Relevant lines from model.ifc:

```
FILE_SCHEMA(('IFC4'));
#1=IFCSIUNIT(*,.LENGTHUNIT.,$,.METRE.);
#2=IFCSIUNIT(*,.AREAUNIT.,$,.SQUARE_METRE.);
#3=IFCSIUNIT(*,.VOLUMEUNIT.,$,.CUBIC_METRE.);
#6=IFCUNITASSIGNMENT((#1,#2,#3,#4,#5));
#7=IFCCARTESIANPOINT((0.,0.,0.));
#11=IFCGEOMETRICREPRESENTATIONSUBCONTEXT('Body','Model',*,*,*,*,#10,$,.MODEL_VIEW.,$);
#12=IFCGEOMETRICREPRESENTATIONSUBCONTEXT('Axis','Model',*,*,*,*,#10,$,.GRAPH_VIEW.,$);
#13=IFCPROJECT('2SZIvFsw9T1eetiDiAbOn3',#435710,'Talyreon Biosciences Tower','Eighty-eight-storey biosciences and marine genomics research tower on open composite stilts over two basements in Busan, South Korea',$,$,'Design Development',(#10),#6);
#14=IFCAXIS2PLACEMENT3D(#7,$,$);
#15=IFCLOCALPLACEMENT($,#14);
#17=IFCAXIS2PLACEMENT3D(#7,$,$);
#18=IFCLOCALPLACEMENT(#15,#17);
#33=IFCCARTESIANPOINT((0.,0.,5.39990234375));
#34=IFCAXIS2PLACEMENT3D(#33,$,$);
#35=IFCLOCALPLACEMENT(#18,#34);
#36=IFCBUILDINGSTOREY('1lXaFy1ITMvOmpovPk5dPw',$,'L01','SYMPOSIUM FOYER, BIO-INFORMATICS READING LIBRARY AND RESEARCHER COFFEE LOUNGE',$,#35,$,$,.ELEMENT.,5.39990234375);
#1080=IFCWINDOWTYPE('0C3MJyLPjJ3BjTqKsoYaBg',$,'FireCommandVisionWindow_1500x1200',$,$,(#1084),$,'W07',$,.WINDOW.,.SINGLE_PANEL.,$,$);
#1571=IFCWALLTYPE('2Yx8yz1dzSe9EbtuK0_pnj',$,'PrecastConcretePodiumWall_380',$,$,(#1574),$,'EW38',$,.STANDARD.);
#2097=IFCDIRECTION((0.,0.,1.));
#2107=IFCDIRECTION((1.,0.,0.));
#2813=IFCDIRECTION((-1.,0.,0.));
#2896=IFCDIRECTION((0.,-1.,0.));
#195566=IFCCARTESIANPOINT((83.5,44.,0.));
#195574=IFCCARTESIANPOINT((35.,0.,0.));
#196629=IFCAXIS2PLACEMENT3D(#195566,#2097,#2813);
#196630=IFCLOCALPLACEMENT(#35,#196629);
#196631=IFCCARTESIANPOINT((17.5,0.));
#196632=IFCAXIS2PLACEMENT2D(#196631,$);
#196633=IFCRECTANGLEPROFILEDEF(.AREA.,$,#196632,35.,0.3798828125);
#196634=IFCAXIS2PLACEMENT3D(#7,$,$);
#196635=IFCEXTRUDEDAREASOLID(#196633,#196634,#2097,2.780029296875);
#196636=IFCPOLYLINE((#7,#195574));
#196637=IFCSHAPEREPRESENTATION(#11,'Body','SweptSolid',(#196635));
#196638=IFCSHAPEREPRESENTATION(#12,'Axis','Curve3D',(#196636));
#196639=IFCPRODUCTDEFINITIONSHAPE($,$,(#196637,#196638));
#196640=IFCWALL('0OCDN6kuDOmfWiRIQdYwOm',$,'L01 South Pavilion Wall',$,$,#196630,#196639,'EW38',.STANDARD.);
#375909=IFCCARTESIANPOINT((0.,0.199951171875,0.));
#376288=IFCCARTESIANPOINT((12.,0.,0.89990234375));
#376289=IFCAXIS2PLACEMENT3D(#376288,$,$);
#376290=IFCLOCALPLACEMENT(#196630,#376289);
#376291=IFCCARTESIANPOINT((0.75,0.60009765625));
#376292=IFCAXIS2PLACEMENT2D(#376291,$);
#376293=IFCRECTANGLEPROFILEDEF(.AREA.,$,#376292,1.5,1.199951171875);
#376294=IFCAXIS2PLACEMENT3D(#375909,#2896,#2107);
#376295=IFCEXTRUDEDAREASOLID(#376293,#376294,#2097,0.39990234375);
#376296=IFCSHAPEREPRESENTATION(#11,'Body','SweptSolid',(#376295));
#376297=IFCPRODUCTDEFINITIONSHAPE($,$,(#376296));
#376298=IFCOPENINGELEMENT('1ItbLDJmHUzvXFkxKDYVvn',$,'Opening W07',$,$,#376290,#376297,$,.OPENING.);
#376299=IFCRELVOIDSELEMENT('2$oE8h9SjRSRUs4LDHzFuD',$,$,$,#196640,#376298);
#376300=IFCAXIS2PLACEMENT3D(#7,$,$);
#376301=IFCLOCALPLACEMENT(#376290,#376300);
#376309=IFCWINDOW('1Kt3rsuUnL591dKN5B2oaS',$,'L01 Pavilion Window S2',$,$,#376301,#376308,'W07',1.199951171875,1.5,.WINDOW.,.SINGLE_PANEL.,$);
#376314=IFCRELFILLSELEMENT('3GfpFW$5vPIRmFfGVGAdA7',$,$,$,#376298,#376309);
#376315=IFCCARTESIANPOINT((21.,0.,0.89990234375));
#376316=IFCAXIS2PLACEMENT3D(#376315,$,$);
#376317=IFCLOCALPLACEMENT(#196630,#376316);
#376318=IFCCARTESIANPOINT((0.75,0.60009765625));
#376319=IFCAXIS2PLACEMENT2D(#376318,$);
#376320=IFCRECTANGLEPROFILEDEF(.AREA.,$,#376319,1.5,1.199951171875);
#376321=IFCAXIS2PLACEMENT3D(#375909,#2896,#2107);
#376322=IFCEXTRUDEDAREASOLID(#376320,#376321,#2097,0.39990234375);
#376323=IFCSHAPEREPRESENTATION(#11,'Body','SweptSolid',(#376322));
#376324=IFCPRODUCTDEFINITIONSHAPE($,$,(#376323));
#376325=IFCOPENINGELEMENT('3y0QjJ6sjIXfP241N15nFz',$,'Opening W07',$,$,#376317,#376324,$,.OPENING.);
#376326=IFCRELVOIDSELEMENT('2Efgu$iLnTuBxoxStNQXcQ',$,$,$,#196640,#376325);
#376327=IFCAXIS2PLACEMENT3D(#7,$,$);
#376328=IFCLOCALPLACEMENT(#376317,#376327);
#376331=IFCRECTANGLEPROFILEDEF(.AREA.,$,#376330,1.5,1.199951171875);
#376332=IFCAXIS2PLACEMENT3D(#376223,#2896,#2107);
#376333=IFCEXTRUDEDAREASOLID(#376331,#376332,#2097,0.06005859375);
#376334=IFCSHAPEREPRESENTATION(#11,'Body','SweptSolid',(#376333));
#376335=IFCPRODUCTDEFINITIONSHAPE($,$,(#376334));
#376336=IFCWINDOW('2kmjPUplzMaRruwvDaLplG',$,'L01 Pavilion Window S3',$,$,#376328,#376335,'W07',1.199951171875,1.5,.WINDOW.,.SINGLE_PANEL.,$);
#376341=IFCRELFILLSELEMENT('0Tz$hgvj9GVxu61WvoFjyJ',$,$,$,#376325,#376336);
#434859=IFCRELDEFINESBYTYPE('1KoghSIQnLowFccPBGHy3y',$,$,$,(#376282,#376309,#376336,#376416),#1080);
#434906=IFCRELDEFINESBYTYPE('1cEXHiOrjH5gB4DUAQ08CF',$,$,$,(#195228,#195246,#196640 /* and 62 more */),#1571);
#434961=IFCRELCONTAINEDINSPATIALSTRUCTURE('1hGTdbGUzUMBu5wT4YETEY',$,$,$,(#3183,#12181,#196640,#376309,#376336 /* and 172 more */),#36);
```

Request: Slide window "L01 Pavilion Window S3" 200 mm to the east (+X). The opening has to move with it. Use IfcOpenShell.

```python
import ifcopenshell
import ifcopenshell.api.geometry
import ifcopenshell.util.placement

model = ifcopenshell.open("model.ifc")

window = model.by_guid("2kmjPUplzMaRruwvDaLplG")
opening = window.FillsVoids[0].RelatingOpeningElement
wall = opening.VoidsElements[0].RelatingBuildingElement

wall_matrix = ifcopenshell.util.placement.get_local_placement(wall.ObjectPlacement)
shift = wall_matrix[:3, 0] * -0.2
before = ifcopenshell.util.placement.get_local_placement(window.ObjectPlacement)[:3, 3].copy()

# The window is placed relative to its opening, so it follows when the opening moves.
matrix = ifcopenshell.util.placement.get_local_placement(opening.ObjectPlacement)
matrix[:3, 3] += shift
ifcopenshell.api.geometry.edit_object_placement(
    model, product=opening, matrix=matrix, is_si=False, should_transform_children=True
)

after = ifcopenshell.util.placement.get_local_placement(window.ObjectPlacement)[:3, 3]
print("window moved by", (after - before).round(3) + 0.0)

model.write("model-out.ifc")
```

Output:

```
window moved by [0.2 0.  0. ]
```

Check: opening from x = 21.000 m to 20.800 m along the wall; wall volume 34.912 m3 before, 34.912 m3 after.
